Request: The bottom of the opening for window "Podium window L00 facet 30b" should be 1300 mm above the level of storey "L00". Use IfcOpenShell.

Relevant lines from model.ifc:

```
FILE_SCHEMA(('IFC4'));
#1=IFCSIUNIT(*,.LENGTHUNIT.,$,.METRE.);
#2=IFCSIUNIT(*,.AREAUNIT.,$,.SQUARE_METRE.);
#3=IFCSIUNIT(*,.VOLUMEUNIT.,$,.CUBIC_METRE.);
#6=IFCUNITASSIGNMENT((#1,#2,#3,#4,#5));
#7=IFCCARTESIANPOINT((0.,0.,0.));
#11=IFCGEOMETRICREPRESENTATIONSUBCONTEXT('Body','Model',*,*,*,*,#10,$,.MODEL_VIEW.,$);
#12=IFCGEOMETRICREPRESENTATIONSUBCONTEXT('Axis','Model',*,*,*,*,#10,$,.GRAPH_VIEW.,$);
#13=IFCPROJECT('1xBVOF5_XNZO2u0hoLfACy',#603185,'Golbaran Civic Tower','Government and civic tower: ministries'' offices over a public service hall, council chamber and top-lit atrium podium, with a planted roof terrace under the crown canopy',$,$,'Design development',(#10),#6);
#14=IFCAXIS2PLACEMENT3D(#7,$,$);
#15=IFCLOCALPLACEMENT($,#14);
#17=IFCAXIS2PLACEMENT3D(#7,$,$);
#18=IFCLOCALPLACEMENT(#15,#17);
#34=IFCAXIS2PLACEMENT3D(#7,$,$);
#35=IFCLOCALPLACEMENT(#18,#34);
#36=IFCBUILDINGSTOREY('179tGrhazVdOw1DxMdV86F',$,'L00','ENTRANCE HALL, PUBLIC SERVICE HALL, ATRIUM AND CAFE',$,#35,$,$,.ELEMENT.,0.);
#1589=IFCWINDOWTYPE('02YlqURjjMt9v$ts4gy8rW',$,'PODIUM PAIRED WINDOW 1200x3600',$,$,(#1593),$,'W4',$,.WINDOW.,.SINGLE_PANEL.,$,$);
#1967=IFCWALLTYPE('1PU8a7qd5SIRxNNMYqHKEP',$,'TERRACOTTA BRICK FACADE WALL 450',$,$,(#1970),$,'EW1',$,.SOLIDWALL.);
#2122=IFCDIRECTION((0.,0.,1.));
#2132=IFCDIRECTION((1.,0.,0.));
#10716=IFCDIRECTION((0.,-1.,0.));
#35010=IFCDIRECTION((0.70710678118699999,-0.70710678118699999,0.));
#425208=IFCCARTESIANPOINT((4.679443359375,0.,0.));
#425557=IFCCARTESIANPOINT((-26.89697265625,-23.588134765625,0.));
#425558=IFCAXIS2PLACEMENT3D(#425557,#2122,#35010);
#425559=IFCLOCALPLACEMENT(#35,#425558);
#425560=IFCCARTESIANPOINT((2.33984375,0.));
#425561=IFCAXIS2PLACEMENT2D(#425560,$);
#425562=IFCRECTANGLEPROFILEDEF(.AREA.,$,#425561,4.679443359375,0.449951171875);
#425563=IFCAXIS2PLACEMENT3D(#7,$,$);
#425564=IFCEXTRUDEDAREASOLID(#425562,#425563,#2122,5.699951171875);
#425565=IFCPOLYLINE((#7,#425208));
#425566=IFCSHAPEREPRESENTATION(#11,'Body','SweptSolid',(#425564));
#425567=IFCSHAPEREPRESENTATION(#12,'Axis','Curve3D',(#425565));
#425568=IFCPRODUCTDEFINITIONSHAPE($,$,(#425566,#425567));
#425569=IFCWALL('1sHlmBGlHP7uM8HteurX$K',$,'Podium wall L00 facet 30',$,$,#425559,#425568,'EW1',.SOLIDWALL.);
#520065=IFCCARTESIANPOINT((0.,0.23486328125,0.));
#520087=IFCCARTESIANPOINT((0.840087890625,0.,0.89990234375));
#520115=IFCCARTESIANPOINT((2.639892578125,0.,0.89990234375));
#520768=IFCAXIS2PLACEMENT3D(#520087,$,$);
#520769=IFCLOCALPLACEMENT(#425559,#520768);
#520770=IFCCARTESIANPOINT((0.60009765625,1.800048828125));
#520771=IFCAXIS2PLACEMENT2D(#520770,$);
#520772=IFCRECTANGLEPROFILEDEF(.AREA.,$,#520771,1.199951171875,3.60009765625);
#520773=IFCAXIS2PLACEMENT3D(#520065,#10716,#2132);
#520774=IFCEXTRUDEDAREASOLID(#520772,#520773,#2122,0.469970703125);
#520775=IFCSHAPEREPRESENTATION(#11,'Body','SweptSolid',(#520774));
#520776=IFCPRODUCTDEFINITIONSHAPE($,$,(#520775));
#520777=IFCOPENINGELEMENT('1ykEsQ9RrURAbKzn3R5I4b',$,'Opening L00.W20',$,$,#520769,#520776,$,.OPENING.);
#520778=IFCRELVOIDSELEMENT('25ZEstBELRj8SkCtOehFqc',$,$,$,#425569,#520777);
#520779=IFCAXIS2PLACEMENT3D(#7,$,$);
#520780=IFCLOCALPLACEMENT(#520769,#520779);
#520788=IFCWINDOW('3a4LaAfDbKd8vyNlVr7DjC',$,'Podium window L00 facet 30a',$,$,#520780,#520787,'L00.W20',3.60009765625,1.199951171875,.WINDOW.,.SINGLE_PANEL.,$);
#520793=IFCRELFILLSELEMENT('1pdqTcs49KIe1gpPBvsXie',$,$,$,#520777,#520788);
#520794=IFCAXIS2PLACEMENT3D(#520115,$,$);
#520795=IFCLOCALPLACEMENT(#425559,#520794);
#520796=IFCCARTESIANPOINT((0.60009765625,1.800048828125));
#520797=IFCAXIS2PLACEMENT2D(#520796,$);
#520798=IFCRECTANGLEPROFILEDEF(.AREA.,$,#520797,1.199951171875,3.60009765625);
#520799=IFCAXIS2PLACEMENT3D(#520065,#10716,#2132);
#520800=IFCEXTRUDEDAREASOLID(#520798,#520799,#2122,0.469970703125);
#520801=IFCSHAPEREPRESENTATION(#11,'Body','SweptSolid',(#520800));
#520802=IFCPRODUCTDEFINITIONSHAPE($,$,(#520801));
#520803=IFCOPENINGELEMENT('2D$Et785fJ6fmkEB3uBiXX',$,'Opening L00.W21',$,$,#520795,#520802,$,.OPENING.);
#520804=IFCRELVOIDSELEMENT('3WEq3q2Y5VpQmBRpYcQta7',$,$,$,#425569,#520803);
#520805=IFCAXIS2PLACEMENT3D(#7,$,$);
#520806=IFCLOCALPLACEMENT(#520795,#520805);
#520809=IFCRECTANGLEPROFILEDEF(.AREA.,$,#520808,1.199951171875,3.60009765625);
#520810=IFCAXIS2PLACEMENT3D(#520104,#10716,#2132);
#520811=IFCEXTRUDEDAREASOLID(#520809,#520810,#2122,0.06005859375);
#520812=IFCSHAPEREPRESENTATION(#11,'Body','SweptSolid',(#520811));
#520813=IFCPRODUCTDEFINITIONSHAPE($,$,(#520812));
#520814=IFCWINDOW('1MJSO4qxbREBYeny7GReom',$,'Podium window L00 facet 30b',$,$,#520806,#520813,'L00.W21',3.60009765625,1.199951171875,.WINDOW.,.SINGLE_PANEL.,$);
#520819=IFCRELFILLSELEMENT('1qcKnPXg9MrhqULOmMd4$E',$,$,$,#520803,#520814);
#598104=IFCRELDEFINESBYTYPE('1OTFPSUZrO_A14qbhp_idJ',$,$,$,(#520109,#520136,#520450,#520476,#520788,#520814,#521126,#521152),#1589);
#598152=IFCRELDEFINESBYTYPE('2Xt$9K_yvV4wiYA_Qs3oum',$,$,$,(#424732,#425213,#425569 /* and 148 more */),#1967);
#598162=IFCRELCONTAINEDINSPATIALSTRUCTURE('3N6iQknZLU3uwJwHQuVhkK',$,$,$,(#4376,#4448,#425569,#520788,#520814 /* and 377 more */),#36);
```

```python
import numpy as np
import ifcopenshell
import ifcopenshell.api.geometry
import ifcopenshell.geom
import ifcopenshell.util.element
import ifcopenshell.util.placement
import ifcopenshell.util.shape
import ifcopenshell.util.unit

model = ifcopenshell.open("model.ifc")
unit_scale = ifcopenshell.util.unit.calculate_unit_scale(model)

window = model.by_guid("1MJSO4qxbREBYeny7GReom")
opening = window.FillsVoids[0].RelatingOpeningElement
storey = ifcopenshell.util.element.get_container(window, ifc_class="IfcBuildingStorey")
level = ifcopenshell.util.placement.get_local_placement(storey.ObjectPlacement)[2, 3]

# The opening's origin need not be at the sill, so measure its lowest point.
shape = ifcopenshell.geom.create_shape(ifcopenshell.geom.settings(), opening)
bottom = ifcopenshell.util.shape.get_shape_bottom_elevation(shape, shape.geometry) / unit_scale
dz = level + 1.3 - bottom

shift = np.array([0.0, 0.0, dz])
# The window is placed relative to its opening, so it follows when the opening moves.
matrix = ifcopenshell.util.placement.get_local_placement(opening.ObjectPlacement)
matrix[:3, 3] += shift
ifcopenshell.api.geometry.edit_object_placement(
    model, product=opening, matrix=matrix, is_si=False, should_transform_children=True
)

print(f"moved by {dz * unit_scale:+.3f} m")

model.write("model-out.ifc")
```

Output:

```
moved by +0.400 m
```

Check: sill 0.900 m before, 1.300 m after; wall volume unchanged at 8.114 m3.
